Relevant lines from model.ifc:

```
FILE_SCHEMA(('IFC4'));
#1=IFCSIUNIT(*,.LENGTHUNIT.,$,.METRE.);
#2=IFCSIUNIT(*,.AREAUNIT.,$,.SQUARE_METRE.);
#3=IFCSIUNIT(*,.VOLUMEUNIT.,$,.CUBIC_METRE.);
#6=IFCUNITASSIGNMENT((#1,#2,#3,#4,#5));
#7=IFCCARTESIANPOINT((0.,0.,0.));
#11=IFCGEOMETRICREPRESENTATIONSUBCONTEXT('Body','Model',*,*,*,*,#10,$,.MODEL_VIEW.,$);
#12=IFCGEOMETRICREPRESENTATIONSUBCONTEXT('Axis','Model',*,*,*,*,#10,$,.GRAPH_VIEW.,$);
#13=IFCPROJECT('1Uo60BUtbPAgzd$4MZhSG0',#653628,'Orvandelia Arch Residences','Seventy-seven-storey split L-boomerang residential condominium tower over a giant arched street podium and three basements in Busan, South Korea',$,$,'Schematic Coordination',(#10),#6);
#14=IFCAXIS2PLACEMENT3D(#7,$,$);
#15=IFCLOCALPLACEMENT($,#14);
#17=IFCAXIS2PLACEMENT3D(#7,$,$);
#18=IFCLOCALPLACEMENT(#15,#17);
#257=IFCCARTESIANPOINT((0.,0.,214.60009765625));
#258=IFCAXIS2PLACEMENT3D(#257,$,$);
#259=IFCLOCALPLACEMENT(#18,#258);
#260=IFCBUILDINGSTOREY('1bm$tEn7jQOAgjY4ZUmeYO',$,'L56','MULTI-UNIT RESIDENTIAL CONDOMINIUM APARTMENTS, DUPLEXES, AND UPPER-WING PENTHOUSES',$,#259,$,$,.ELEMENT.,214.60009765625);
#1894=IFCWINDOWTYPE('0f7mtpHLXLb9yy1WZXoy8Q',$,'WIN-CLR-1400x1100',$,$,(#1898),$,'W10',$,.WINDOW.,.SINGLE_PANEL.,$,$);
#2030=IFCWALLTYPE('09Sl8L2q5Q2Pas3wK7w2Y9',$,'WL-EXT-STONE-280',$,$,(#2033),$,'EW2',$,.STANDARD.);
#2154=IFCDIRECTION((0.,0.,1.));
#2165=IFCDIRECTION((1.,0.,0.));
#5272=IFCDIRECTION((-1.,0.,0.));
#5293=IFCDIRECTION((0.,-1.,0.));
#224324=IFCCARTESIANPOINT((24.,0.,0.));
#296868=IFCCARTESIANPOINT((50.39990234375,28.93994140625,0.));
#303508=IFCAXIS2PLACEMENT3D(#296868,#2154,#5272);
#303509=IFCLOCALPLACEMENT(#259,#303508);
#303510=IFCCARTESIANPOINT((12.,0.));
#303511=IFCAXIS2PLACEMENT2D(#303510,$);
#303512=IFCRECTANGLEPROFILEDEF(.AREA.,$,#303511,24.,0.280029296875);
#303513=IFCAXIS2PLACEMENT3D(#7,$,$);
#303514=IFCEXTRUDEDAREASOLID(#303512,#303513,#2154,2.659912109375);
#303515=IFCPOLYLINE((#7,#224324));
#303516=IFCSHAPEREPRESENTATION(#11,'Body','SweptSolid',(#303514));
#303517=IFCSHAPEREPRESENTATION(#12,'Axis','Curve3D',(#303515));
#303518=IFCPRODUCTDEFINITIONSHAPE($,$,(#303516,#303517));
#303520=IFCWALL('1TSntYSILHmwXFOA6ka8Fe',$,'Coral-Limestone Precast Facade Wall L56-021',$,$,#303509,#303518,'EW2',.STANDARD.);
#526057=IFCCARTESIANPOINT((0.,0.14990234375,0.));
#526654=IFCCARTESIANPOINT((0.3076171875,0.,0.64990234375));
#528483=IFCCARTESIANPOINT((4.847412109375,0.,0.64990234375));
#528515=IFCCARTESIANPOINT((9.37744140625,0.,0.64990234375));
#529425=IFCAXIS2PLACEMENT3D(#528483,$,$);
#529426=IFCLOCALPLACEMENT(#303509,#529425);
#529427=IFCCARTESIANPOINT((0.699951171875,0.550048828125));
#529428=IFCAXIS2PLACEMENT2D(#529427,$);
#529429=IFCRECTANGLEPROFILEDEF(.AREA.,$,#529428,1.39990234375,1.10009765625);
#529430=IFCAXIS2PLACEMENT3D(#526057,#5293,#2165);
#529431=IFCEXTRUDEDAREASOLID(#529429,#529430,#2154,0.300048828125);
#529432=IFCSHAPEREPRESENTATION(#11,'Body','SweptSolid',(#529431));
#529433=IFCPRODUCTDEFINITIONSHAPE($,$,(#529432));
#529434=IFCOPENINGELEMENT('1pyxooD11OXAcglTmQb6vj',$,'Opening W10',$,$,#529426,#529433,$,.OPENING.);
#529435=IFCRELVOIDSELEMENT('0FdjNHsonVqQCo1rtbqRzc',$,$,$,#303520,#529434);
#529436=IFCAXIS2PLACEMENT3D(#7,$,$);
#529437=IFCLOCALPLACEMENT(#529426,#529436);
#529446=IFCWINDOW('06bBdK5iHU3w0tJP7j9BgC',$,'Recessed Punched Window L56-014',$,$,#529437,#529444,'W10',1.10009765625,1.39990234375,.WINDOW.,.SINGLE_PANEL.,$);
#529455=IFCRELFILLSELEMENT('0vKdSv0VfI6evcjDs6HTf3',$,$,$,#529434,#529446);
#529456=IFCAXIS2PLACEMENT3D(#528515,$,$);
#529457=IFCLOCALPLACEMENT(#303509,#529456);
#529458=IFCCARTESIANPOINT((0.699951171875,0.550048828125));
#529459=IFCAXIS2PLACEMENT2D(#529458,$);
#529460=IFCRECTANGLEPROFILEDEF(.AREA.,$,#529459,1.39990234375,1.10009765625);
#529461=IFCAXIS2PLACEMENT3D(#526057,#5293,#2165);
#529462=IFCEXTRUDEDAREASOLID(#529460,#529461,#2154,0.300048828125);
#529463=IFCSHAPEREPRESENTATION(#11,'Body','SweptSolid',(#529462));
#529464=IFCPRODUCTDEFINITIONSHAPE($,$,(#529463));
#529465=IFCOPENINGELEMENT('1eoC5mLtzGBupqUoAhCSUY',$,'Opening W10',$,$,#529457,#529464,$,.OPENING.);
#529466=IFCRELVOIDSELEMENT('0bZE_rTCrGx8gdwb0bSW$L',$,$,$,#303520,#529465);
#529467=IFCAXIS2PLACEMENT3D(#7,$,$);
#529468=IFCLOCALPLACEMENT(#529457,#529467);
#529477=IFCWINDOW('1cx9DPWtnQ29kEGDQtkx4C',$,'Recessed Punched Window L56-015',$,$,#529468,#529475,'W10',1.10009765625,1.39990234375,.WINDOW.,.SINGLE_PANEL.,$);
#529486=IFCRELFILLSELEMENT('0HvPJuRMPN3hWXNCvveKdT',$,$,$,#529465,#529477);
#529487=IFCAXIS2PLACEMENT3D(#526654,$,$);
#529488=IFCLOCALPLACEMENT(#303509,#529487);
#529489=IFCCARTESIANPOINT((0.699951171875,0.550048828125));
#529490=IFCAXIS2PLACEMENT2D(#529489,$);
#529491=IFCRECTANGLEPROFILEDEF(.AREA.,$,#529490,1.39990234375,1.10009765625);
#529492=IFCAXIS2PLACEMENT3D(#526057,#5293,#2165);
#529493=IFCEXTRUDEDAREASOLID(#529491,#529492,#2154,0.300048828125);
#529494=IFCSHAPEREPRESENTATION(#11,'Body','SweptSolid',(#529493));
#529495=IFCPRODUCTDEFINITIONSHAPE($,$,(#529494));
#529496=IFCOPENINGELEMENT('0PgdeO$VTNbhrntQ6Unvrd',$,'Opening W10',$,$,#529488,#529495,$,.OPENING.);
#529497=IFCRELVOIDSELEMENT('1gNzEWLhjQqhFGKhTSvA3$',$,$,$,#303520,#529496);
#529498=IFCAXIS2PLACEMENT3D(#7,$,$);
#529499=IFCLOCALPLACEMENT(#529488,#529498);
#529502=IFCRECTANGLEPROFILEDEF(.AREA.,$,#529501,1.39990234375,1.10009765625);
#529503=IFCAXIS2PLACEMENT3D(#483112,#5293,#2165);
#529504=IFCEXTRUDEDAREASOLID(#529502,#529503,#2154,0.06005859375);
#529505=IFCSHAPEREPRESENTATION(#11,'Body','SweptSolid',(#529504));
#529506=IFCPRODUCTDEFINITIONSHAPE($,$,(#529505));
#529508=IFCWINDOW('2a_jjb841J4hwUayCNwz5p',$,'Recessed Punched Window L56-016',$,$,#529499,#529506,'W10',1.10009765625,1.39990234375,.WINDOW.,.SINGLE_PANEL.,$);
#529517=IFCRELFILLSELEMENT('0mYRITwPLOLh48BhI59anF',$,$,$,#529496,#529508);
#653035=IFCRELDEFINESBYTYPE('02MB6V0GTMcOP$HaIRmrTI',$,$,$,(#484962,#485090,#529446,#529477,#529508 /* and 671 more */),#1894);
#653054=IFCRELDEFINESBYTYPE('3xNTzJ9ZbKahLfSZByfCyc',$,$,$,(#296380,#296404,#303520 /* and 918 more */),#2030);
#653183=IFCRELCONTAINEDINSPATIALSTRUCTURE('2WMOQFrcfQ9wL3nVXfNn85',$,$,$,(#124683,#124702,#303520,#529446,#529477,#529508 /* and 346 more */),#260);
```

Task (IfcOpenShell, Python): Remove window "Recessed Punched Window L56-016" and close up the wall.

```python
import ifcopenshell
import ifcopenshell.api.feature
import ifcopenshell.api.root
import ifcopenshell.geom
import ifcopenshell.util.shape

model = ifcopenshell.open("model.ifc")
settings = ifcopenshell.geom.settings()


def volume(element):
    """Net volume in cubic metres, openings subtracted."""
    shape = ifcopenshell.geom.create_shape(settings, element)
    return ifcopenshell.util.shape.get_volume(shape.geometry)


window = model.by_id(529508)
opening = window.FillsVoids[0].RelatingOpeningElement
wall = opening.VoidsElements[0].RelatingBuildingElement
before = volume(wall)

ifcopenshell.api.root.remove_product(model, product=window)
ifcopenshell.api.feature.remove_feature(model, feature=opening)

after = volume(wall)

print(f"wall volume {before:.3f} -> {after:.3f} m3")

model.write("model_edited.ifc")
```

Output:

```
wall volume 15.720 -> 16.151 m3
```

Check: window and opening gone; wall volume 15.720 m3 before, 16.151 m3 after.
